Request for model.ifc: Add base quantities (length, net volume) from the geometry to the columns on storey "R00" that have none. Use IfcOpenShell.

First a look at what the model holds.

```python
import ifcopenshell
import ifcopenshell.util.element
import ifcopenshell.util.unit

model = ifcopenshell.open("model.ifc")
print(model.schema)
for unit_type in ("LENGTHUNIT", "AREAUNIT", "VOLUMEUNIT"):
    print(unit_type, ifcopenshell.util.unit.calculate_unit_scale(model, unit_type))
storey = next(s for s in model.by_type("IfcBuildingStorey") if s.Name == "R00")
columns = [e for e in ifcopenshell.util.element.get_decomposition(storey) if e.is_a("IfcColumn")]
for e in sorted(columns, key=lambda e: e.id()):
    print(e.id(), e.is_a(), e.Name, list(ifcopenshell.util.element.get_psets(e, qtos_only=True)), sep=" | ")
```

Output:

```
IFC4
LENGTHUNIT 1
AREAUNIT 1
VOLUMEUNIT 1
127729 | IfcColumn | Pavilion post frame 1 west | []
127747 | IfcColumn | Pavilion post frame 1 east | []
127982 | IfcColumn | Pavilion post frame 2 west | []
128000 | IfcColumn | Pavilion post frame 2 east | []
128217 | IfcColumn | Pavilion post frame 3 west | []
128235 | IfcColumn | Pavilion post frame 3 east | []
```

```python
import ifcopenshell
import ifcopenshell.api.pset
import ifcopenshell.geom
import ifcopenshell.util.element
import ifcopenshell.util.shape
import ifcopenshell.util.unit

model = ifcopenshell.open("model.ifc")
unit_scale = ifcopenshell.util.unit.calculate_unit_scale(model)
volume_scale = ifcopenshell.util.unit.calculate_unit_scale(model, "VOLUMEUNIT")
settings = ifcopenshell.geom.settings()

storey = next(s for s in model.by_type("IfcBuildingStorey") if s.Name == "R00")
columns = [e for e in ifcopenshell.util.element.get_decomposition(storey) if e.is_a("IfcColumn")]

for e in sorted(columns, key=lambda e: e.id()):
    if ifcopenshell.util.element.get_psets(e, qtos_only=True, should_inherit=False):
        continue
    # Geometry comes back in metres, in the element's own axes.
    shape = ifcopenshell.geom.create_shape(settings, e)
    values = {
        "Length": ifcopenshell.util.shape.get_z(shape.geometry) / unit_scale,
        "NetVolume": ifcopenshell.util.shape.get_volume(shape.geometry) / volume_scale,
    }
    qto = ifcopenshell.api.pset.add_qto(model, product=e, name="Qto_ColumnBaseQuantities")
    ifcopenshell.api.pset.edit_qto(model, qto=qto, properties=values)
    print(e.id(), {k: round(v, 3) for k, v in values.items()})

model.write("model_v2.ifc")
```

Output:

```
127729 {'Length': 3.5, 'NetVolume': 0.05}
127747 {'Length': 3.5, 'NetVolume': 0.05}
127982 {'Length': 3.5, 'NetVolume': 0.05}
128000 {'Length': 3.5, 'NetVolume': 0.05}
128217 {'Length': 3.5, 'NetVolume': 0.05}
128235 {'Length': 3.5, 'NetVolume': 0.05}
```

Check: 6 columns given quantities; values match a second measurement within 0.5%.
